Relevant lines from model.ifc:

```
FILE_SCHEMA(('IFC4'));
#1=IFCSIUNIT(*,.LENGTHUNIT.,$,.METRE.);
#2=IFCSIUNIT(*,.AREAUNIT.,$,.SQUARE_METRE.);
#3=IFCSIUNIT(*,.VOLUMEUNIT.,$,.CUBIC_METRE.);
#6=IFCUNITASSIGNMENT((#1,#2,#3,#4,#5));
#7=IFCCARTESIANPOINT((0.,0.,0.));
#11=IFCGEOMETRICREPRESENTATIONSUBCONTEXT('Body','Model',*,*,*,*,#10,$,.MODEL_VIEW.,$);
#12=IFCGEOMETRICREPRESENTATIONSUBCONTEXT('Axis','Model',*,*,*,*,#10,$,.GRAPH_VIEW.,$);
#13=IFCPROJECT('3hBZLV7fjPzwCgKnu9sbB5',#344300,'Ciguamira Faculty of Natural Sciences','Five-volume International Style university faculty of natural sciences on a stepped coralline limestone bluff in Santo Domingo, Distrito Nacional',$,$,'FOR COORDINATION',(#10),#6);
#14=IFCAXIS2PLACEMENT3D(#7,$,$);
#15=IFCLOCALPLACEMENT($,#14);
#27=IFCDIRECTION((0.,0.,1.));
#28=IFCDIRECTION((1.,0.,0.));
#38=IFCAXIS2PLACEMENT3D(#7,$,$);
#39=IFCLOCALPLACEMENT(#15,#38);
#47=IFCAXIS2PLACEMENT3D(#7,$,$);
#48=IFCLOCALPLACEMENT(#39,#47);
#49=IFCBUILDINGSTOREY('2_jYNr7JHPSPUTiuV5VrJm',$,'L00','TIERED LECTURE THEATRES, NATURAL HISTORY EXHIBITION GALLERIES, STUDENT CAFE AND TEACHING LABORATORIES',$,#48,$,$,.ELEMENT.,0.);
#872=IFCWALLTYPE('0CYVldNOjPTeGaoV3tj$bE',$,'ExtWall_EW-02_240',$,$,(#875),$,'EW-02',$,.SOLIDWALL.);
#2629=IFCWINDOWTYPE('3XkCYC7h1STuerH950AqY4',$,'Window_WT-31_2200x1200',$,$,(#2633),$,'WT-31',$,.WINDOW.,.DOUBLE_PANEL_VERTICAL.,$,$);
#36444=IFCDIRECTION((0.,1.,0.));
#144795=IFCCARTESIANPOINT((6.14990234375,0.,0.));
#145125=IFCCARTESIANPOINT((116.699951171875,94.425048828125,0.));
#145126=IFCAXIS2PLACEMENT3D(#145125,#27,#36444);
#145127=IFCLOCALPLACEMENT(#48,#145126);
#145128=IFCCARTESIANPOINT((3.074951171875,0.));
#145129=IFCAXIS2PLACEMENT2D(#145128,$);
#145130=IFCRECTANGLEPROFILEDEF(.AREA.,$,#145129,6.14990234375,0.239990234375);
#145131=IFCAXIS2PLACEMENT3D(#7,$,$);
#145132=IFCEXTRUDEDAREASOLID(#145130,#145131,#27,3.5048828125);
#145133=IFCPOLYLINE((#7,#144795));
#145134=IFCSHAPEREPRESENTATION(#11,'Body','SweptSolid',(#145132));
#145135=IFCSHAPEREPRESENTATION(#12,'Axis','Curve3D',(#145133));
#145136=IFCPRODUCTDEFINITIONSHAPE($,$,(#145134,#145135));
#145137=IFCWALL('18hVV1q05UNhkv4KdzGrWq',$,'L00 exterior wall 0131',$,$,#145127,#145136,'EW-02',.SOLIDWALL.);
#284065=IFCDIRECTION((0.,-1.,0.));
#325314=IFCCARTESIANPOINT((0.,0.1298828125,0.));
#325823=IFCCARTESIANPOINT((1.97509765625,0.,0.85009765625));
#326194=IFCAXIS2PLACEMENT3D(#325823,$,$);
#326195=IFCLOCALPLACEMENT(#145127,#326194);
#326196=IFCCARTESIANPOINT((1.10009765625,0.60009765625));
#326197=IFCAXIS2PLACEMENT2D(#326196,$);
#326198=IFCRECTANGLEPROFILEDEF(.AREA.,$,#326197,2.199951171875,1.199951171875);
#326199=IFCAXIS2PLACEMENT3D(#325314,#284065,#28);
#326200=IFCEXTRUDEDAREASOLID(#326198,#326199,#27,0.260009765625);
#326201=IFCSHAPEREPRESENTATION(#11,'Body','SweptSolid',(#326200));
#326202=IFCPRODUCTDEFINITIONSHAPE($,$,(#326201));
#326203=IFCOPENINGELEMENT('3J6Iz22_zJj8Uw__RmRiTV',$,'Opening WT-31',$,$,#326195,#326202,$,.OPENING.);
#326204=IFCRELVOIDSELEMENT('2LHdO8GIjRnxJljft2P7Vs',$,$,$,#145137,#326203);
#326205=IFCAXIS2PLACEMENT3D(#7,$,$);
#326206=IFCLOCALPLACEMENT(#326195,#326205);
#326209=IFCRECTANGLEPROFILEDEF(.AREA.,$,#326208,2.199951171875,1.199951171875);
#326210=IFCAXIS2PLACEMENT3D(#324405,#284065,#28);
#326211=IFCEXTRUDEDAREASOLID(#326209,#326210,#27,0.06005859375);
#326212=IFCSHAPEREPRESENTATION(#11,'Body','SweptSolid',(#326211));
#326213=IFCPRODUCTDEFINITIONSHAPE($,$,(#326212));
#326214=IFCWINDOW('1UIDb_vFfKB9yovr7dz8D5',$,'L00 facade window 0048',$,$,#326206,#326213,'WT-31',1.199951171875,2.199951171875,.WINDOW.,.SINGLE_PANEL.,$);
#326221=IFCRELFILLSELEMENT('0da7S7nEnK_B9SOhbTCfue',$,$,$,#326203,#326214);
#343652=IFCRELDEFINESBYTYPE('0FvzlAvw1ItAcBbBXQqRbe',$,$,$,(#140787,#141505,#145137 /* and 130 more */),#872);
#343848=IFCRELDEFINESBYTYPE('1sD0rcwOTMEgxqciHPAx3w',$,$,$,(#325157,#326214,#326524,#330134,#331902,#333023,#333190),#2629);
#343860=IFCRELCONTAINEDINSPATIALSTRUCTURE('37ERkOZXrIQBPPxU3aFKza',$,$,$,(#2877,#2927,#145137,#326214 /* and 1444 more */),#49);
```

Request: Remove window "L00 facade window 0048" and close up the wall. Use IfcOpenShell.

```python
import ifcopenshell
import ifcopenshell.api.feature
import ifcopenshell.api.root
import ifcopenshell.geom
import ifcopenshell.util.shape

model = ifcopenshell.open("model.ifc")
settings = ifcopenshell.geom.settings()


def volume(element):
    """Net volume in cubic metres, openings subtracted."""
    shape = ifcopenshell.geom.create_shape(settings, element)
    return ifcopenshell.util.shape.get_volume(shape.geometry)


window = model.by_guid("1UIDb_vFfKB9yovr7dz8D5")
opening = window.FillsVoids[0].RelatingOpeningElement
wall = opening.VoidsElements[0].RelatingBuildingElement
before = volume(wall)

ifcopenshell.api.root.remove_product(model, product=window)
ifcopenshell.api.feature.remove_feature(model, feature=opening)

after = volume(wall)

print(f"wall volume {before:.3f} -> {after:.3f} m3")

model.write("model_updated.ifc")
```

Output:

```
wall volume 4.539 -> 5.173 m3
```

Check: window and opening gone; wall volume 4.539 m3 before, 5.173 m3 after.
